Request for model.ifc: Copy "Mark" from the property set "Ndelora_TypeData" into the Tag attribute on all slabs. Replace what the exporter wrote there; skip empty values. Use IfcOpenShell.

First a look at what the model holds.

```python
import ifcopenshell
import ifcopenshell.util.element

model = ifcopenshell.open("model.ifc")
print(model.schema)
slabs = model.by_type("IfcSlab")
print(len(slabs), "slabs")
for e in slabs[:8]:
    source = ifcopenshell.util.element.get_pset(e, "Ndelora_TypeData", "Mark")
    target = e.Tag
    print(e.id(), repr(source), repr(target), sep=" | ")
```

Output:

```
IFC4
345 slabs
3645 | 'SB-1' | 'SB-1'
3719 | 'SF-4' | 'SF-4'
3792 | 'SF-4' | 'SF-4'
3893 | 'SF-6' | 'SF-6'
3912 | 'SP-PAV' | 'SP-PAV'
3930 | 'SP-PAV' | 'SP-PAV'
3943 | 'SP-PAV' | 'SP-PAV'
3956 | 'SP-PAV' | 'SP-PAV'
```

```python
import ifcopenshell
import ifcopenshell.util.element

model = ifcopenshell.open("model.ifc")

count = 0
for e in model.by_type("IfcSlab"):
    value = ifcopenshell.util.element.get_pset(e, "Ndelora_TypeData", "Mark")
    current = e.Tag
    if not value or not value.strip() or current == value:
        continue
    e.Tag = value
    count += 1

print(count, "slabs updated")

model.write("model_v2.ifc")
```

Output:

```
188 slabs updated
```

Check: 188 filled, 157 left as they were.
